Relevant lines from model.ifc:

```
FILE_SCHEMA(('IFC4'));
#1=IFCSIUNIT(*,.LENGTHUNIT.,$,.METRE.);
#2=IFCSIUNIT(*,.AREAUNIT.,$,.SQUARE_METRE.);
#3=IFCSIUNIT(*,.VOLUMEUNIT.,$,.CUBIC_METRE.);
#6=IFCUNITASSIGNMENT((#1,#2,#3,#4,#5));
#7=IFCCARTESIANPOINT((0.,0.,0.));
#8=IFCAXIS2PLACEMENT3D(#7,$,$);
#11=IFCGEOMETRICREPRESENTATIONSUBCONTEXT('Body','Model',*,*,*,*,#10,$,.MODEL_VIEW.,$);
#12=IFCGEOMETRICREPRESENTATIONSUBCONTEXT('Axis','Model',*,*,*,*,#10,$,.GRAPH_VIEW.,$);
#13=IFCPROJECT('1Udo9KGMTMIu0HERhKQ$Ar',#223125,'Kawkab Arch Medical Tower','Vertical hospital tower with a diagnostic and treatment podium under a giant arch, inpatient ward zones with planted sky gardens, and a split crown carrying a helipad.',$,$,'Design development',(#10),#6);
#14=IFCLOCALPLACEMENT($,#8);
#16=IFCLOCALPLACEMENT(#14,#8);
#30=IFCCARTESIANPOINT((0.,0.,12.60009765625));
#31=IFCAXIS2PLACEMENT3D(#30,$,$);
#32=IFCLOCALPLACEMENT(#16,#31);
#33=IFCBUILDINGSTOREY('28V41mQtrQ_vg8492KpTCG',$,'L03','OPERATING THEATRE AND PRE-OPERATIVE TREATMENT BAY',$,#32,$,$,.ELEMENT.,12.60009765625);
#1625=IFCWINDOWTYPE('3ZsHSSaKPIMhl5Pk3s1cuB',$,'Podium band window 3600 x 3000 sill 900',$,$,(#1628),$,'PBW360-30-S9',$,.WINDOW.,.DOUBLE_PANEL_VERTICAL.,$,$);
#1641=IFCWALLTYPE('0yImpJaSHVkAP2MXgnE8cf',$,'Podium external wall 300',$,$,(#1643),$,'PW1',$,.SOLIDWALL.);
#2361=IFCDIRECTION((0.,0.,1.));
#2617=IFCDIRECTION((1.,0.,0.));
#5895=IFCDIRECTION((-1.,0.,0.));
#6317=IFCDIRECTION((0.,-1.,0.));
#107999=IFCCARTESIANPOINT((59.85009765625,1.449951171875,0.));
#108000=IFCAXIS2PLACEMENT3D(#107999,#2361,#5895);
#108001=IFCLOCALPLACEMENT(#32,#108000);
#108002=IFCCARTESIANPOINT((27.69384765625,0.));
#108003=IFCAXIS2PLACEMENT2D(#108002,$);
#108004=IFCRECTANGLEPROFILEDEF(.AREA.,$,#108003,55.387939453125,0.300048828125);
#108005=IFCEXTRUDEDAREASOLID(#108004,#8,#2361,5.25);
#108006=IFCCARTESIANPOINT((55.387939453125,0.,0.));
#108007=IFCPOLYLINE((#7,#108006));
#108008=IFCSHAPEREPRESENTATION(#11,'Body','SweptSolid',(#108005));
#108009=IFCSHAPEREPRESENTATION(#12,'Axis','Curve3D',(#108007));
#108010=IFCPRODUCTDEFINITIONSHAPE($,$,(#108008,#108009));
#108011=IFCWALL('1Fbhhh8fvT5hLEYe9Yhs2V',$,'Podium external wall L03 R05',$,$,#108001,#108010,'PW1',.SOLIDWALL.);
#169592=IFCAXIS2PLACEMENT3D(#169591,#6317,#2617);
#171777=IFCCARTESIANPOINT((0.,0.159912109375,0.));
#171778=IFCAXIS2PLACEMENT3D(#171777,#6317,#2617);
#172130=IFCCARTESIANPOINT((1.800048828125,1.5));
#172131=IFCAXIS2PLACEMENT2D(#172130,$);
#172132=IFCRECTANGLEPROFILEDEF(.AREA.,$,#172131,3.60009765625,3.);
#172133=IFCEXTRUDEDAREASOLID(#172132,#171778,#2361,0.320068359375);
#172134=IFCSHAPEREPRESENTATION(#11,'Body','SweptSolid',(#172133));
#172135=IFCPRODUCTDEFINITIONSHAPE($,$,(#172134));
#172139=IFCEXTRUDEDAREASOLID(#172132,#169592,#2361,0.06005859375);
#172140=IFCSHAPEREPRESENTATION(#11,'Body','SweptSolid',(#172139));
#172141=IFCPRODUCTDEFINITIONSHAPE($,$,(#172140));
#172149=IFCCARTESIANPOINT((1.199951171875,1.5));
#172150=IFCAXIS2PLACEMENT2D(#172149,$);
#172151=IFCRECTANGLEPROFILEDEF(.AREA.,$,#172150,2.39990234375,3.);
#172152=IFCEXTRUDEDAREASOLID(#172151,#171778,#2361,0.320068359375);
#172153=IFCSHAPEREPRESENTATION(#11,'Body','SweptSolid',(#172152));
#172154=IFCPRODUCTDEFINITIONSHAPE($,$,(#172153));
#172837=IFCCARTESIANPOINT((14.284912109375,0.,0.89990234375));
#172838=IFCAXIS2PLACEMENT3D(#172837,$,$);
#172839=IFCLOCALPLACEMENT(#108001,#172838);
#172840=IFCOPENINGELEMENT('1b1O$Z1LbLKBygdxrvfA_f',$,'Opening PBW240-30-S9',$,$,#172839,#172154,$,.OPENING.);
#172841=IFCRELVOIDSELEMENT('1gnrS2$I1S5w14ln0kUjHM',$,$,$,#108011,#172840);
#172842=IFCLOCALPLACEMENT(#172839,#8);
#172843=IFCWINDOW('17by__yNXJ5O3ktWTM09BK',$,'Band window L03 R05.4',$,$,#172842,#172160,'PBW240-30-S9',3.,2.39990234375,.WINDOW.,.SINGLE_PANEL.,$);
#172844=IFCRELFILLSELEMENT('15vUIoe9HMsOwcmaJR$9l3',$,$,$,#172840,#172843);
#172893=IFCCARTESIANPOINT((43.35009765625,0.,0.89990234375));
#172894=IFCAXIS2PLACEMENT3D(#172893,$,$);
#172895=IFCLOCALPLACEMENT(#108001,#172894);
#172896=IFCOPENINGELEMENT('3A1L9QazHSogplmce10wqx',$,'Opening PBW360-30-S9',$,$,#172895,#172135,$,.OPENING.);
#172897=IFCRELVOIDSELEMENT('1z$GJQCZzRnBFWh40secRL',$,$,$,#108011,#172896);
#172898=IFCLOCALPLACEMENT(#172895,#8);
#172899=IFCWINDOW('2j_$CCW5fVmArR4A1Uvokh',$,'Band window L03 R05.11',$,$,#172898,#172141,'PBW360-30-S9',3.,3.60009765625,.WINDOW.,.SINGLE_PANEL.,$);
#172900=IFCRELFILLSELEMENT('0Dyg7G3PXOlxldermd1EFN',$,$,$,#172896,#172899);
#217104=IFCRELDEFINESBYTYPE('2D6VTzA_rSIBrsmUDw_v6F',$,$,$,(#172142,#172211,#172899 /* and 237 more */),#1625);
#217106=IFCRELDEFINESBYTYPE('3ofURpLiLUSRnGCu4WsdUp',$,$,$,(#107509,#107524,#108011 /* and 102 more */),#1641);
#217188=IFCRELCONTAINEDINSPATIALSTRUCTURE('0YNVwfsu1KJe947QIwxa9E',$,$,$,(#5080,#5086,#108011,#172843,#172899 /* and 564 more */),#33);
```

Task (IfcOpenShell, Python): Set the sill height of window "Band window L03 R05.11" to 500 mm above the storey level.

```python
import numpy as np
import ifcopenshell
import ifcopenshell.api.geometry
import ifcopenshell.geom
import ifcopenshell.util.element
import ifcopenshell.util.placement
import ifcopenshell.util.shape
import ifcopenshell.util.unit

model = ifcopenshell.open("model.ifc")
unit_scale = ifcopenshell.util.unit.calculate_unit_scale(model)

window = model.by_guid("2j_$CCW5fVmArR4A1Uvokh")
opening = window.FillsVoids[0].RelatingOpeningElement
storey = ifcopenshell.util.element.get_container(window, ifc_class="IfcBuildingStorey")
level = ifcopenshell.util.placement.get_local_placement(storey.ObjectPlacement)[2, 3]

# The opening's origin need not be at the sill, so measure its lowest point.
shape = ifcopenshell.geom.create_shape(ifcopenshell.geom.settings(), opening)
bottom = ifcopenshell.util.shape.get_shape_bottom_elevation(shape, shape.geometry) / unit_scale
dz = level + 0.5 / unit_scale - bottom

shift = np.array([0.0, 0.0, dz])
# The window is placed relative to its opening, so it follows when the opening moves.
matrix = ifcopenshell.util.placement.get_local_placement(opening.ObjectPlacement)
matrix[:3, 3] += shift
ifcopenshell.api.geometry.edit_object_placement(
    model, product=opening, matrix=matrix, is_si=False, should_transform_children=True
)

print(f"moved by {dz * unit_scale:+.3f} m")

model.write("model-out.ifc")
```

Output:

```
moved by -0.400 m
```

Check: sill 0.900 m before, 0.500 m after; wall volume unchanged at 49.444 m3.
